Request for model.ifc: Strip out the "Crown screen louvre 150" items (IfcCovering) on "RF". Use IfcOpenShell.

First a look at what the model holds.

```python
import ifcopenshell
import ifcopenshell.util.element

model = ifcopenshell.open("model.ifc")
print(model.schema)
storey = next(s for s in model.by_type("IfcBuildingStorey") if s.Name == "RF")
coverings = [e for e in ifcopenshell.util.element.get_decomposition(storey) if e.is_a("IfcCovering")]
seen = {}
for e in coverings:
    element_type = ifcopenshell.util.element.get_type(e)
    name = element_type.Name if element_type not in (None, e) else None
    seen[name] = seen.get(name, 0) + 1
for name, count in sorted(seen.items(), key=str):
    print(count, "x", name)
```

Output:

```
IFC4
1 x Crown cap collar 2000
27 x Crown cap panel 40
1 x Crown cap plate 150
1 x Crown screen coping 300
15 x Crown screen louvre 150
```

```python
import ifcopenshell
import ifcopenshell.api.root
import ifcopenshell.util.element

model = ifcopenshell.open("model.ifc")

storey = next(s for s in model.by_type("IfcBuildingStorey") if s.Name == "RF")
coverings = [e for e in ifcopenshell.util.element.get_decomposition(storey) if e.is_a("IfcCovering")]
targets = [e for e in coverings if (t := ifcopenshell.util.element.get_type(e)) not in (None, e) and t.Name == "Crown screen louvre 150"]

for e in targets:
    ifcopenshell.api.root.remove_product(model, product=e)
print(len(targets), "removed")

model.write("model_rev.ifc")
```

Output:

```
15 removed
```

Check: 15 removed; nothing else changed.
